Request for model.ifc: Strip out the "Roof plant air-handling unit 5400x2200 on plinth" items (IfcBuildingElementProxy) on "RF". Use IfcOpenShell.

First a look at what the model holds.

```python
import ifcopenshell
import ifcopenshell.util.element

model = ifcopenshell.open("model.ifc")
print(model.schema)
storey = next(s for s in model.by_type("IfcBuildingStorey") if s.Name == "RF")
proxies = [e for e in ifcopenshell.util.element.get_decomposition(storey) if e.is_a("IfcBuildingElementProxy")]
seen = {}
for e in proxies:
    element_type = ifcopenshell.util.element.get_type(e)
    name = element_type.Name if element_type not in (None, e) else None
    seen[name] = seen.get(name, 0) + 1
for name, count in sorted(seen.items(), key=str):
    print(count, "x", name)
```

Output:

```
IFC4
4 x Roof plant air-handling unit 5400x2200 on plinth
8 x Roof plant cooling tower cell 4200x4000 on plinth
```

```python
import ifcopenshell
import ifcopenshell.api.root
import ifcopenshell.util.element

model = ifcopenshell.open("model.ifc")

storey = next(s for s in model.by_type("IfcBuildingStorey") if s.Name == "RF")
proxies = [e for e in ifcopenshell.util.element.get_decomposition(storey) if e.is_a("IfcBuildingElementProxy")]
targets = [e for e in proxies if (t := ifcopenshell.util.element.get_type(e)) not in (None, e) and t.Name == "Roof plant air-handling unit 5400x2200 on plinth"]

for e in targets:
    ifcopenshell.api.root.remove_product(model, product=e)
print(len(targets), "removed")

model.write("model_updated.ifc")
```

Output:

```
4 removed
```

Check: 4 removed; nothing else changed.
